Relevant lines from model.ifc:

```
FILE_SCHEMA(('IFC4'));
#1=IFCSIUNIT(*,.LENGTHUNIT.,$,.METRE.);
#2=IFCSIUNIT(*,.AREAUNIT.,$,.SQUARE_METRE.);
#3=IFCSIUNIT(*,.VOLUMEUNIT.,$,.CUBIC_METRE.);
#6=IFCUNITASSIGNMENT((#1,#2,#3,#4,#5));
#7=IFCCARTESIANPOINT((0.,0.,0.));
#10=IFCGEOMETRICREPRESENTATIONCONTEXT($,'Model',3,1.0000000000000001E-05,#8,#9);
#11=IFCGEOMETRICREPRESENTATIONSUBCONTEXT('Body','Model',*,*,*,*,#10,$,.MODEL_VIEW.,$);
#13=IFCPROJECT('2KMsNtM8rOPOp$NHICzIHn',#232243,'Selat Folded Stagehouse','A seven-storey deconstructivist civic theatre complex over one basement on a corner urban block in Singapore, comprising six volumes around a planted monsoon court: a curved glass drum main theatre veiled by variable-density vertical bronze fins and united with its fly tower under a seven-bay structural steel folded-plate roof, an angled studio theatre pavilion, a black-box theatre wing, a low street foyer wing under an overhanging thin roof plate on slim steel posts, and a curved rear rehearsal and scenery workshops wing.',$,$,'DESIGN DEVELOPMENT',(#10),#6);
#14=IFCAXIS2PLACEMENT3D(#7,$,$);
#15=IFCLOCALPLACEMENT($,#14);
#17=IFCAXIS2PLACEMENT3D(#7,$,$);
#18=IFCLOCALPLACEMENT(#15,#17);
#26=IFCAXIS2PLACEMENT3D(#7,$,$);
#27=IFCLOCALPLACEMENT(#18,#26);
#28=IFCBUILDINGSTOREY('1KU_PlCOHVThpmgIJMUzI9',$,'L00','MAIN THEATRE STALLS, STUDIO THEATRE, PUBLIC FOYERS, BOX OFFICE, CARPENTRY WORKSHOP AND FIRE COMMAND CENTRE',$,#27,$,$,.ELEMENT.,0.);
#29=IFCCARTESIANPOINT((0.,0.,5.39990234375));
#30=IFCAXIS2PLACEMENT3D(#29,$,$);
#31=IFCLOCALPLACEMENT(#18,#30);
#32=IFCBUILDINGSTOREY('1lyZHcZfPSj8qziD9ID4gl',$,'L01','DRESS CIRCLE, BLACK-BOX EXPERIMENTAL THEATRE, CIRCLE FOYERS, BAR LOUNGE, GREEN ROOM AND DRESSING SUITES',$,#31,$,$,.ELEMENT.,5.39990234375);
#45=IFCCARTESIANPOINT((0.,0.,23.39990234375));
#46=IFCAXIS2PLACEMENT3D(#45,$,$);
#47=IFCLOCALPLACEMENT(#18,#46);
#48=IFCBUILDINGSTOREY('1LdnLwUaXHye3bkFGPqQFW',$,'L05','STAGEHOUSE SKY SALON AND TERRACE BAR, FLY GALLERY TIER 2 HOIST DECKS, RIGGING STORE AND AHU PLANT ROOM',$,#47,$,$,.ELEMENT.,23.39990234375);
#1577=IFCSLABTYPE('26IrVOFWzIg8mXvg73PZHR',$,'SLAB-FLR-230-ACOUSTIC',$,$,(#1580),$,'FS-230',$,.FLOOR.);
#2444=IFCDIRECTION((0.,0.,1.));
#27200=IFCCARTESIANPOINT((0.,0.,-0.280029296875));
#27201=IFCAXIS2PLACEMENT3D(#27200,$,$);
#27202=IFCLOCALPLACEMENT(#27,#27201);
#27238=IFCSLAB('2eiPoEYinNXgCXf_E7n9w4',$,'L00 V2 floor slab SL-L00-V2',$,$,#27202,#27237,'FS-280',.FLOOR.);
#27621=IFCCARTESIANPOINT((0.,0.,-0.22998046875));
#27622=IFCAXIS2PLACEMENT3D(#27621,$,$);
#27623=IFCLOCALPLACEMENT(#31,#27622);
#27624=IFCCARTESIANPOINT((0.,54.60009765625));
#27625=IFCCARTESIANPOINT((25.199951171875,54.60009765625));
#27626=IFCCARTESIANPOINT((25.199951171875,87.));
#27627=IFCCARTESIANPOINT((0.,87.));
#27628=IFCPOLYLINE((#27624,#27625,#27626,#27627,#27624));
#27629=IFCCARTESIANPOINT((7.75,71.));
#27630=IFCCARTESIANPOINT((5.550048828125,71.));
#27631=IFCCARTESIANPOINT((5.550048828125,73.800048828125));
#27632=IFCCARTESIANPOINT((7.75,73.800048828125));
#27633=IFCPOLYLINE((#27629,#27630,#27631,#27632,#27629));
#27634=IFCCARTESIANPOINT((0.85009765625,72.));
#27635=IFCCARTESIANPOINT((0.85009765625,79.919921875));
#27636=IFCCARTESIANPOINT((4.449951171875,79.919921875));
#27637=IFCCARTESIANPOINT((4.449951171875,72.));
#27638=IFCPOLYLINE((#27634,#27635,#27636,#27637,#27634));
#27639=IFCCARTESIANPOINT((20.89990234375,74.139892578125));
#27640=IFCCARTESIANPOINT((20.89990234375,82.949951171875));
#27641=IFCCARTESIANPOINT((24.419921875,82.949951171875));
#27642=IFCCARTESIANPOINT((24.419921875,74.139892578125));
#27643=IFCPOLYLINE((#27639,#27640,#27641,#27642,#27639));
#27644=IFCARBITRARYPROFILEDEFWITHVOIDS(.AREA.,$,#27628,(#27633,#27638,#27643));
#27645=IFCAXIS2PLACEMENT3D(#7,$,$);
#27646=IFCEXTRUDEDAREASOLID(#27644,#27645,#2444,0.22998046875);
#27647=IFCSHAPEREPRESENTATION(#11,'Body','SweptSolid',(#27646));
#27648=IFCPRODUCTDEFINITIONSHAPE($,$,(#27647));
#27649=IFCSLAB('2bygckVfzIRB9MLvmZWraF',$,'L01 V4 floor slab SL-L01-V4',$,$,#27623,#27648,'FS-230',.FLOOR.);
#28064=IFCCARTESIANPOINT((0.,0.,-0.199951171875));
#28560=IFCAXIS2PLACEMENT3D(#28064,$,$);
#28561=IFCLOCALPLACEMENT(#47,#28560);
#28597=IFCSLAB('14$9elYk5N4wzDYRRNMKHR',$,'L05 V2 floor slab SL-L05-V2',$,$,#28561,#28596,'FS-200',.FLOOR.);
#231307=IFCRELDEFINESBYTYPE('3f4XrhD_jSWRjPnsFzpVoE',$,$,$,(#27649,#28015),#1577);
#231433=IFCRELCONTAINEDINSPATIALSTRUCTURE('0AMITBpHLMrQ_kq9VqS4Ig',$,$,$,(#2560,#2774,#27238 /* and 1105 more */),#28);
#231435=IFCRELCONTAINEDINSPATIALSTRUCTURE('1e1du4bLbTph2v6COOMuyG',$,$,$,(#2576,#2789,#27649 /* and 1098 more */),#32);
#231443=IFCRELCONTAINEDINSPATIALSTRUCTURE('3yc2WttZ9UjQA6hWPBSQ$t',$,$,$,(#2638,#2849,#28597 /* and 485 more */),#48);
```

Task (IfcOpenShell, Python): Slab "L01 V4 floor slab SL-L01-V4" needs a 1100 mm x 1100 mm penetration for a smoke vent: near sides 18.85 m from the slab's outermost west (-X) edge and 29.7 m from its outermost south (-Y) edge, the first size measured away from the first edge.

```python
import numpy as np
import ifcopenshell
import ifcopenshell.api.feature
import ifcopenshell.api.geometry
import ifcopenshell.api.root
import ifcopenshell.geom
import ifcopenshell.util.placement
import ifcopenshell.util.representation
import ifcopenshell.util.shape
import ifcopenshell.util.unit

model = ifcopenshell.open("model.ifc")
unit_scale = ifcopenshell.util.unit.calculate_unit_scale(model)
settings = ifcopenshell.geom.settings()


def volume(element):
    """Net volume in cubic metres, openings subtracted."""
    shape = ifcopenshell.geom.create_shape(settings, element)
    return ifcopenshell.util.shape.get_volume(shape.geometry)


slab = model.by_guid("2bygckVfzIRB9MLvmZWraF")
before = volume(slab)

# Extent in the slab's own axes, in metres. The edges named are its -X and -Y sides.
slab_shape = ifcopenshell.geom.create_shape(settings, slab)
vertices = ifcopenshell.util.shape.get_vertices(slab_shape.geometry)
x_min, y_min, bottom = vertices.min(axis=0)
top = vertices[:, 2].max()

opening = ifcopenshell.api.root.create_entity(model, ifc_class="IfcOpeningElement", name="Smoke vent opening", predefined_type="OPENING")
context = ifcopenshell.util.representation.get_context(model, "Model", "Body", "MODEL_VIEW")
width, depth = 1.1, 1.1
outline = [(0.0, 0.0), (width, 0.0), (width, depth), (0.0, depth), (0.0, 0.0)]
# Overshoot both faces by 50 mm so the cut is clean.
shape = ifcopenshell.api.geometry.add_slab_representation(
    model, context=context, depth=top - bottom + 0.1, polyline=outline
)
ifcopenshell.api.geometry.assign_representation(model, product=opening, representation=shape)

matrix = ifcopenshell.util.placement.get_local_placement(slab.ObjectPlacement)
matrix[:, 3] = matrix @ np.append(np.array([x_min + 18.85, y_min + 29.7, bottom - 0.05]) / unit_scale, 1.0)
ifcopenshell.api.geometry.edit_object_placement(model, product=opening, matrix=matrix, is_si=False)
ifcopenshell.api.feature.add_feature(model, feature=opening, element=slab)

after = volume(slab)

print(f"slab volume {before:.3f} -> {after:.3f} m3")

model.write("model_v2.ifc")
```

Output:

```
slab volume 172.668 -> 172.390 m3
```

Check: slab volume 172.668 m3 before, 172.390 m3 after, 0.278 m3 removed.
